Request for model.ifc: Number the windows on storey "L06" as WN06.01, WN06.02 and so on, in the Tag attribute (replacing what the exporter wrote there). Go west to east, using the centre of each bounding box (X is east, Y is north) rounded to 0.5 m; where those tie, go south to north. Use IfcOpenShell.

First a look at what the model holds.

```python
import ifcopenshell
import ifcopenshell.util.element
import ifcopenshell.util.placement

model = ifcopenshell.open("model.ifc")
print(model.schema)
storey = next(s for s in model.by_type("IfcBuildingStorey") if s.Name == "L06")
windows = [e for e in ifcopenshell.util.element.get_decomposition(storey) if e.is_a("IfcWindow")]
for e in sorted(windows, key=lambda e: e.id()):
    origin = ifcopenshell.util.placement.get_local_placement(e.ObjectPlacement)[:3, 3]
    print(e.id(), e.Tag, e.Name, origin.round(2) + 0.0, sep=" | ")
```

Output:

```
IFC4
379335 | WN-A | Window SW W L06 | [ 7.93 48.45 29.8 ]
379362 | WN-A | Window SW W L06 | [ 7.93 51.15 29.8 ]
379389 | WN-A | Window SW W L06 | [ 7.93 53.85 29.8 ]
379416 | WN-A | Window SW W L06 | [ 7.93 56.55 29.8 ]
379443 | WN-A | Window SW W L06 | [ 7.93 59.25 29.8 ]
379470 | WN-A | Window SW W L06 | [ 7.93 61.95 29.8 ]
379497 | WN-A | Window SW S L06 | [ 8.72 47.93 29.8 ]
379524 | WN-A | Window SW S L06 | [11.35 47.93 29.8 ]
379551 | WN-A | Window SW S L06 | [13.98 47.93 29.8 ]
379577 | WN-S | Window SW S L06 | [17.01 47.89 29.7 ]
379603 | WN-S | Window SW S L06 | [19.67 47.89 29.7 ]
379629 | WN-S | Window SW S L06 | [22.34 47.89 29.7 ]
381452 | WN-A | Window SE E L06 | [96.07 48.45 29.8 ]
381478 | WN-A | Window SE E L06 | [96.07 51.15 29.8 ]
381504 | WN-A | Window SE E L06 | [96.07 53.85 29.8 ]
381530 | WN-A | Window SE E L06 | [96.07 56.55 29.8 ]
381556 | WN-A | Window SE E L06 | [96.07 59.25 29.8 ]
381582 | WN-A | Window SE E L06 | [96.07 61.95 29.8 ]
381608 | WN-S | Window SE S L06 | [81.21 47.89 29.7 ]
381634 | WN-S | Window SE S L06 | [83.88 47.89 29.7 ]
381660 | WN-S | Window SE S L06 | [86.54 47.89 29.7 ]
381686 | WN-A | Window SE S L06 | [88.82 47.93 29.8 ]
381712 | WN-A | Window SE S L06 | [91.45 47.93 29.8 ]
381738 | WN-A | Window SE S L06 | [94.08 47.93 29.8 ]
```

```python
import ifcopenshell
import ifcopenshell.geom
import ifcopenshell.util.element
import ifcopenshell.util.shape

model = ifcopenshell.open("model.ifc")
settings = ifcopenshell.geom.settings()
settings.set("use-world-coords", True)


def centre(element):
    shape = ifcopenshell.geom.create_shape(settings, element)
    return ifcopenshell.util.shape.get_bbox_centroid(shape.geometry)


storey = next(s for s in model.by_type("IfcBuildingStorey") if s.Name == "L06")
windows = [e for e in ifcopenshell.util.element.get_decomposition(storey) if e.is_a("IfcWindow")]

# Insertion points can sit at a corner or the storey origin, so sort by the geometry (in metres).
centres = {e: centre(e) for e in windows}
windows.sort(key=lambda e: (round(centres[e][0] / 0.5), centres[e][1]))

for i, e in enumerate(windows, start=1):
    number = f"WN06.{i:02d}"
    e.Tag = number
    print(e.id(), number)

model.write("model-out.ifc")
```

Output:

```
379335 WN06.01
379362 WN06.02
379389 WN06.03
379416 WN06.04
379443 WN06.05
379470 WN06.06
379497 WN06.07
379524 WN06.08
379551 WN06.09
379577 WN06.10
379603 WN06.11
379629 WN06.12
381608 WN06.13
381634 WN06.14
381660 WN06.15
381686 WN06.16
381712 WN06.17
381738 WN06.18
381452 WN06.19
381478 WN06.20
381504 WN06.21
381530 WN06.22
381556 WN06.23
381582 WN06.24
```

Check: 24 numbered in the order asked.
